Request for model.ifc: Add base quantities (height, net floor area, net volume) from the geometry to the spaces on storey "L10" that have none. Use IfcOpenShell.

First a look at what the model holds.

```python
import ifcopenshell
import ifcopenshell.util.element
import ifcopenshell.util.unit

model = ifcopenshell.open("model.ifc")
print(model.schema)
for unit_type in ("LENGTHUNIT", "AREAUNIT", "VOLUMEUNIT"):
    print(unit_type, ifcopenshell.util.unit.calculate_unit_scale(model, unit_type))
storey = next(s for s in model.by_type("IfcBuildingStorey") if s.Name == "L10")
spaces = [e for e in ifcopenshell.util.element.get_decomposition(storey) if e.is_a("IfcSpace")]
for e in sorted(spaces, key=lambda e: e.id()):
    print(e.id(), e.is_a(), e.Name, list(ifcopenshell.util.element.get_psets(e, qtos_only=True)), sep=" | ")
```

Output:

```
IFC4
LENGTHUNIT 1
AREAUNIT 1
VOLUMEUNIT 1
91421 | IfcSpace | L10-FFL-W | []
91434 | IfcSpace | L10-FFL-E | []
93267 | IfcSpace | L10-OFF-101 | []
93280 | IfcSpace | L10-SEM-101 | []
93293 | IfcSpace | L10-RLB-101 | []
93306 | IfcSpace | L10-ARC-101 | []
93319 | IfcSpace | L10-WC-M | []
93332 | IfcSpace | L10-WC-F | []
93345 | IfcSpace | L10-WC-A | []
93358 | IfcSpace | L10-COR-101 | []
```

```python
import ifcopenshell
import ifcopenshell.api.pset
import ifcopenshell.geom
import ifcopenshell.util.element
import ifcopenshell.util.shape
import ifcopenshell.util.unit

model = ifcopenshell.open("model.ifc")
unit_scale = ifcopenshell.util.unit.calculate_unit_scale(model)
area_scale = ifcopenshell.util.unit.calculate_unit_scale(model, "AREAUNIT")
volume_scale = ifcopenshell.util.unit.calculate_unit_scale(model, "VOLUMEUNIT")
settings = ifcopenshell.geom.settings()

storey = next(s for s in model.by_type("IfcBuildingStorey") if s.Name == "L10")
spaces = [e for e in ifcopenshell.util.element.get_decomposition(storey) if e.is_a("IfcSpace")]

for e in sorted(spaces, key=lambda e: e.id()):
    if ifcopenshell.util.element.get_psets(e, qtos_only=True, should_inherit=False):
        continue
    # Geometry comes back in metres, in the element's own axes.
    shape = ifcopenshell.geom.create_shape(settings, e)
    values = {
        "Height": ifcopenshell.util.shape.get_z(shape.geometry) / unit_scale,
        "NetFloorArea": ifcopenshell.util.shape.get_footprint_area(shape.geometry) / area_scale,
        "NetVolume": ifcopenshell.util.shape.get_volume(shape.geometry) / volume_scale,
    }
    qto = ifcopenshell.api.pset.add_qto(model, product=e, name="Qto_SpaceBaseQuantities")
    ifcopenshell.api.pset.edit_qto(model, qto=qto, properties=values)
    print(e.id(), {k: round(v, 3) for k, v in values.items()})

model.write("model_edited.ifc")
```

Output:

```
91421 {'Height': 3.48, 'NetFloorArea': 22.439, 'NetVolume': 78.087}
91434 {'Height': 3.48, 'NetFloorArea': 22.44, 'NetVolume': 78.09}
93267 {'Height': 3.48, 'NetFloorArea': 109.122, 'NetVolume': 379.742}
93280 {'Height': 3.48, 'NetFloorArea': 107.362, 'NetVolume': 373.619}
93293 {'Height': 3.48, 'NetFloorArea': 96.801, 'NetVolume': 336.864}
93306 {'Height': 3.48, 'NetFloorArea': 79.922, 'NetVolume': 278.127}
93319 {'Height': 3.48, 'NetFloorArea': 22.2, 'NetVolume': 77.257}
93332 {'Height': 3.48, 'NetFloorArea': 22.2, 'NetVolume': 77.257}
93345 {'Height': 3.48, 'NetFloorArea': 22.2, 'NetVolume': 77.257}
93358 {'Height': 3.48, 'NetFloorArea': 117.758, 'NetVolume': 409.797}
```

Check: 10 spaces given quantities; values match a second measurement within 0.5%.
